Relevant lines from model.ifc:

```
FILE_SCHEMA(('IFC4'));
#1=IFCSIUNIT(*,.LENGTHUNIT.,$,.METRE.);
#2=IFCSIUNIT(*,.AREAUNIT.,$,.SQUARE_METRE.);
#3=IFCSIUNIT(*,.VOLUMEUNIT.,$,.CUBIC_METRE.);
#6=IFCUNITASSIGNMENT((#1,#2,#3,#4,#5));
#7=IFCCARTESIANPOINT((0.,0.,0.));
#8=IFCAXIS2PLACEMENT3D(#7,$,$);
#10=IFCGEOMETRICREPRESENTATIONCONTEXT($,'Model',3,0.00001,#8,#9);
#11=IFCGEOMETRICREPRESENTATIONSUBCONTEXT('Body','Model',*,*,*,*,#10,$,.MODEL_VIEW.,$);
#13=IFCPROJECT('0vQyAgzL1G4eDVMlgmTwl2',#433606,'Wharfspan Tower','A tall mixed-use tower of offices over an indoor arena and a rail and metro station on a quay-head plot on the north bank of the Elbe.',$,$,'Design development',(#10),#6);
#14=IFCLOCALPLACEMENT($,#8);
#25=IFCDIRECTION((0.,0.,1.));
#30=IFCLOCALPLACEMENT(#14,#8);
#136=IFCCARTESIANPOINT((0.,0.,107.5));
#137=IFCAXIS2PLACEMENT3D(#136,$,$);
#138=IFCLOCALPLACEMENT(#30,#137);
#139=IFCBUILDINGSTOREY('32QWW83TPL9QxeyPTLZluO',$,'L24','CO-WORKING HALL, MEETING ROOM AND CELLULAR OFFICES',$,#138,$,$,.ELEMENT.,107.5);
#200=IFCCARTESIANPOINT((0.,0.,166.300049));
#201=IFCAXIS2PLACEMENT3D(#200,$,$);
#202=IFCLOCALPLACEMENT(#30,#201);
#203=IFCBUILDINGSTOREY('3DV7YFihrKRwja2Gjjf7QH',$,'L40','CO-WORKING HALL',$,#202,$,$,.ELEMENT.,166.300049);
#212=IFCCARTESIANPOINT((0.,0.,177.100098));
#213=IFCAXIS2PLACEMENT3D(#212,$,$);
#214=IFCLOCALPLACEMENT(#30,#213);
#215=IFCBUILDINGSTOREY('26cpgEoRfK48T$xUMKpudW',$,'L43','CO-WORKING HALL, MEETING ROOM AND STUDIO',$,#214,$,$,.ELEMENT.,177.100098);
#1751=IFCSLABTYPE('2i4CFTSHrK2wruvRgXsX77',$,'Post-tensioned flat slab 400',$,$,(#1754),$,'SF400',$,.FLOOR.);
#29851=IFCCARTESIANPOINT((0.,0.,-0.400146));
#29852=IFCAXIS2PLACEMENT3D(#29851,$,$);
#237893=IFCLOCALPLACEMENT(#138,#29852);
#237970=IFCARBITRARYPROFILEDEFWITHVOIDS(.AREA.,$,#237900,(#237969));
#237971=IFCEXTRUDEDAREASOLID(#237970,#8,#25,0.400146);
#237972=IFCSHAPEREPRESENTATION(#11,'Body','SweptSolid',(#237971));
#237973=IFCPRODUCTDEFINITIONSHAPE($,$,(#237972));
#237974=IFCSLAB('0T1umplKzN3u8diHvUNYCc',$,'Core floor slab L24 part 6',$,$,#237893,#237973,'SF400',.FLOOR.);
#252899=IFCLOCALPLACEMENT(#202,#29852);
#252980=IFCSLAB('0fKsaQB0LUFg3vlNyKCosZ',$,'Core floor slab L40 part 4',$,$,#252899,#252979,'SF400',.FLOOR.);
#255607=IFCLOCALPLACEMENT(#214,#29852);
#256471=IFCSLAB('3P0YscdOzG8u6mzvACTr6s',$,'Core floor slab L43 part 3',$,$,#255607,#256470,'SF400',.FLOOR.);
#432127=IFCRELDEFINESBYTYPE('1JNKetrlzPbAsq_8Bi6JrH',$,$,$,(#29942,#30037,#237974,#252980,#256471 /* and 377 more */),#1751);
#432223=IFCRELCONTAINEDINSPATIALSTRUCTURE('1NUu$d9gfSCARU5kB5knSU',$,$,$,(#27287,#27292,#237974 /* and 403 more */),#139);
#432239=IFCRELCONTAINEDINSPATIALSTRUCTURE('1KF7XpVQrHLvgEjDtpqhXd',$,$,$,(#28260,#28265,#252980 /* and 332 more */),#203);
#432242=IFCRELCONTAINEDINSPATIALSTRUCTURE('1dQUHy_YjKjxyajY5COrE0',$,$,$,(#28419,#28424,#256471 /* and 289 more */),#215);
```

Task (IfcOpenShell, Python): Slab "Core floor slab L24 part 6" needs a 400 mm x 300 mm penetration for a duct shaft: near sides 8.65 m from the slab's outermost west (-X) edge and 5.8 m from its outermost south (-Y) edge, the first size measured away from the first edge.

```python
import numpy as np
import ifcopenshell
import ifcopenshell.api.feature
import ifcopenshell.api.geometry
import ifcopenshell.api.root
import ifcopenshell.geom
import ifcopenshell.util.placement
import ifcopenshell.util.representation
import ifcopenshell.util.shape
import ifcopenshell.util.unit

model = ifcopenshell.open("model.ifc")
unit_scale = ifcopenshell.util.unit.calculate_unit_scale(model)
settings = ifcopenshell.geom.settings()


def volume(element):
    """Net volume in cubic metres, openings subtracted."""
    shape = ifcopenshell.geom.create_shape(settings, element)
    return ifcopenshell.util.shape.get_volume(shape.geometry)


slab = model.by_guid("0T1umplKzN3u8diHvUNYCc")
before = volume(slab)

# Extent in the slab's own axes, in metres. The edges named are its -X and -Y sides.
slab_shape = ifcopenshell.geom.create_shape(settings, slab)
vertices = ifcopenshell.util.shape.get_vertices(slab_shape.geometry)
x_min, y_min, bottom = vertices.min(axis=0)
top = vertices[:, 2].max()

opening = ifcopenshell.api.root.create_entity(model, ifc_class="IfcOpeningElement", name="Duct shaft opening", predefined_type="OPENING")
context = ifcopenshell.util.representation.get_context(model, "Model", "Body", "MODEL_VIEW")
width, depth = 0.4, 0.3
outline = [(0.0, 0.0), (width, 0.0), (width, depth), (0.0, depth), (0.0, 0.0)]
# Overshoot both faces by 50 mm so the cut is clean.
shape = ifcopenshell.api.geometry.add_slab_representation(
    model, context=context, depth=top - bottom + 0.1, polyline=outline
)
ifcopenshell.api.geometry.assign_representation(model, product=opening, representation=shape)

matrix = ifcopenshell.util.placement.get_local_placement(slab.ObjectPlacement)
matrix[:, 3] = matrix @ np.append(np.array([x_min + 8.65, y_min + 5.8, bottom - 0.05]) / unit_scale, 1.0)
ifcopenshell.api.geometry.edit_object_placement(model, product=opening, matrix=matrix, is_si=False)
ifcopenshell.api.feature.add_feature(model, feature=opening, element=slab)

after = volume(slab)

print(f"slab volume {before:.3f} -> {after:.3f} m3")

model.write("model_v2.ifc")
```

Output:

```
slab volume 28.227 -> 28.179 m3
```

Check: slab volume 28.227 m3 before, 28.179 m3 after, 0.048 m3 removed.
